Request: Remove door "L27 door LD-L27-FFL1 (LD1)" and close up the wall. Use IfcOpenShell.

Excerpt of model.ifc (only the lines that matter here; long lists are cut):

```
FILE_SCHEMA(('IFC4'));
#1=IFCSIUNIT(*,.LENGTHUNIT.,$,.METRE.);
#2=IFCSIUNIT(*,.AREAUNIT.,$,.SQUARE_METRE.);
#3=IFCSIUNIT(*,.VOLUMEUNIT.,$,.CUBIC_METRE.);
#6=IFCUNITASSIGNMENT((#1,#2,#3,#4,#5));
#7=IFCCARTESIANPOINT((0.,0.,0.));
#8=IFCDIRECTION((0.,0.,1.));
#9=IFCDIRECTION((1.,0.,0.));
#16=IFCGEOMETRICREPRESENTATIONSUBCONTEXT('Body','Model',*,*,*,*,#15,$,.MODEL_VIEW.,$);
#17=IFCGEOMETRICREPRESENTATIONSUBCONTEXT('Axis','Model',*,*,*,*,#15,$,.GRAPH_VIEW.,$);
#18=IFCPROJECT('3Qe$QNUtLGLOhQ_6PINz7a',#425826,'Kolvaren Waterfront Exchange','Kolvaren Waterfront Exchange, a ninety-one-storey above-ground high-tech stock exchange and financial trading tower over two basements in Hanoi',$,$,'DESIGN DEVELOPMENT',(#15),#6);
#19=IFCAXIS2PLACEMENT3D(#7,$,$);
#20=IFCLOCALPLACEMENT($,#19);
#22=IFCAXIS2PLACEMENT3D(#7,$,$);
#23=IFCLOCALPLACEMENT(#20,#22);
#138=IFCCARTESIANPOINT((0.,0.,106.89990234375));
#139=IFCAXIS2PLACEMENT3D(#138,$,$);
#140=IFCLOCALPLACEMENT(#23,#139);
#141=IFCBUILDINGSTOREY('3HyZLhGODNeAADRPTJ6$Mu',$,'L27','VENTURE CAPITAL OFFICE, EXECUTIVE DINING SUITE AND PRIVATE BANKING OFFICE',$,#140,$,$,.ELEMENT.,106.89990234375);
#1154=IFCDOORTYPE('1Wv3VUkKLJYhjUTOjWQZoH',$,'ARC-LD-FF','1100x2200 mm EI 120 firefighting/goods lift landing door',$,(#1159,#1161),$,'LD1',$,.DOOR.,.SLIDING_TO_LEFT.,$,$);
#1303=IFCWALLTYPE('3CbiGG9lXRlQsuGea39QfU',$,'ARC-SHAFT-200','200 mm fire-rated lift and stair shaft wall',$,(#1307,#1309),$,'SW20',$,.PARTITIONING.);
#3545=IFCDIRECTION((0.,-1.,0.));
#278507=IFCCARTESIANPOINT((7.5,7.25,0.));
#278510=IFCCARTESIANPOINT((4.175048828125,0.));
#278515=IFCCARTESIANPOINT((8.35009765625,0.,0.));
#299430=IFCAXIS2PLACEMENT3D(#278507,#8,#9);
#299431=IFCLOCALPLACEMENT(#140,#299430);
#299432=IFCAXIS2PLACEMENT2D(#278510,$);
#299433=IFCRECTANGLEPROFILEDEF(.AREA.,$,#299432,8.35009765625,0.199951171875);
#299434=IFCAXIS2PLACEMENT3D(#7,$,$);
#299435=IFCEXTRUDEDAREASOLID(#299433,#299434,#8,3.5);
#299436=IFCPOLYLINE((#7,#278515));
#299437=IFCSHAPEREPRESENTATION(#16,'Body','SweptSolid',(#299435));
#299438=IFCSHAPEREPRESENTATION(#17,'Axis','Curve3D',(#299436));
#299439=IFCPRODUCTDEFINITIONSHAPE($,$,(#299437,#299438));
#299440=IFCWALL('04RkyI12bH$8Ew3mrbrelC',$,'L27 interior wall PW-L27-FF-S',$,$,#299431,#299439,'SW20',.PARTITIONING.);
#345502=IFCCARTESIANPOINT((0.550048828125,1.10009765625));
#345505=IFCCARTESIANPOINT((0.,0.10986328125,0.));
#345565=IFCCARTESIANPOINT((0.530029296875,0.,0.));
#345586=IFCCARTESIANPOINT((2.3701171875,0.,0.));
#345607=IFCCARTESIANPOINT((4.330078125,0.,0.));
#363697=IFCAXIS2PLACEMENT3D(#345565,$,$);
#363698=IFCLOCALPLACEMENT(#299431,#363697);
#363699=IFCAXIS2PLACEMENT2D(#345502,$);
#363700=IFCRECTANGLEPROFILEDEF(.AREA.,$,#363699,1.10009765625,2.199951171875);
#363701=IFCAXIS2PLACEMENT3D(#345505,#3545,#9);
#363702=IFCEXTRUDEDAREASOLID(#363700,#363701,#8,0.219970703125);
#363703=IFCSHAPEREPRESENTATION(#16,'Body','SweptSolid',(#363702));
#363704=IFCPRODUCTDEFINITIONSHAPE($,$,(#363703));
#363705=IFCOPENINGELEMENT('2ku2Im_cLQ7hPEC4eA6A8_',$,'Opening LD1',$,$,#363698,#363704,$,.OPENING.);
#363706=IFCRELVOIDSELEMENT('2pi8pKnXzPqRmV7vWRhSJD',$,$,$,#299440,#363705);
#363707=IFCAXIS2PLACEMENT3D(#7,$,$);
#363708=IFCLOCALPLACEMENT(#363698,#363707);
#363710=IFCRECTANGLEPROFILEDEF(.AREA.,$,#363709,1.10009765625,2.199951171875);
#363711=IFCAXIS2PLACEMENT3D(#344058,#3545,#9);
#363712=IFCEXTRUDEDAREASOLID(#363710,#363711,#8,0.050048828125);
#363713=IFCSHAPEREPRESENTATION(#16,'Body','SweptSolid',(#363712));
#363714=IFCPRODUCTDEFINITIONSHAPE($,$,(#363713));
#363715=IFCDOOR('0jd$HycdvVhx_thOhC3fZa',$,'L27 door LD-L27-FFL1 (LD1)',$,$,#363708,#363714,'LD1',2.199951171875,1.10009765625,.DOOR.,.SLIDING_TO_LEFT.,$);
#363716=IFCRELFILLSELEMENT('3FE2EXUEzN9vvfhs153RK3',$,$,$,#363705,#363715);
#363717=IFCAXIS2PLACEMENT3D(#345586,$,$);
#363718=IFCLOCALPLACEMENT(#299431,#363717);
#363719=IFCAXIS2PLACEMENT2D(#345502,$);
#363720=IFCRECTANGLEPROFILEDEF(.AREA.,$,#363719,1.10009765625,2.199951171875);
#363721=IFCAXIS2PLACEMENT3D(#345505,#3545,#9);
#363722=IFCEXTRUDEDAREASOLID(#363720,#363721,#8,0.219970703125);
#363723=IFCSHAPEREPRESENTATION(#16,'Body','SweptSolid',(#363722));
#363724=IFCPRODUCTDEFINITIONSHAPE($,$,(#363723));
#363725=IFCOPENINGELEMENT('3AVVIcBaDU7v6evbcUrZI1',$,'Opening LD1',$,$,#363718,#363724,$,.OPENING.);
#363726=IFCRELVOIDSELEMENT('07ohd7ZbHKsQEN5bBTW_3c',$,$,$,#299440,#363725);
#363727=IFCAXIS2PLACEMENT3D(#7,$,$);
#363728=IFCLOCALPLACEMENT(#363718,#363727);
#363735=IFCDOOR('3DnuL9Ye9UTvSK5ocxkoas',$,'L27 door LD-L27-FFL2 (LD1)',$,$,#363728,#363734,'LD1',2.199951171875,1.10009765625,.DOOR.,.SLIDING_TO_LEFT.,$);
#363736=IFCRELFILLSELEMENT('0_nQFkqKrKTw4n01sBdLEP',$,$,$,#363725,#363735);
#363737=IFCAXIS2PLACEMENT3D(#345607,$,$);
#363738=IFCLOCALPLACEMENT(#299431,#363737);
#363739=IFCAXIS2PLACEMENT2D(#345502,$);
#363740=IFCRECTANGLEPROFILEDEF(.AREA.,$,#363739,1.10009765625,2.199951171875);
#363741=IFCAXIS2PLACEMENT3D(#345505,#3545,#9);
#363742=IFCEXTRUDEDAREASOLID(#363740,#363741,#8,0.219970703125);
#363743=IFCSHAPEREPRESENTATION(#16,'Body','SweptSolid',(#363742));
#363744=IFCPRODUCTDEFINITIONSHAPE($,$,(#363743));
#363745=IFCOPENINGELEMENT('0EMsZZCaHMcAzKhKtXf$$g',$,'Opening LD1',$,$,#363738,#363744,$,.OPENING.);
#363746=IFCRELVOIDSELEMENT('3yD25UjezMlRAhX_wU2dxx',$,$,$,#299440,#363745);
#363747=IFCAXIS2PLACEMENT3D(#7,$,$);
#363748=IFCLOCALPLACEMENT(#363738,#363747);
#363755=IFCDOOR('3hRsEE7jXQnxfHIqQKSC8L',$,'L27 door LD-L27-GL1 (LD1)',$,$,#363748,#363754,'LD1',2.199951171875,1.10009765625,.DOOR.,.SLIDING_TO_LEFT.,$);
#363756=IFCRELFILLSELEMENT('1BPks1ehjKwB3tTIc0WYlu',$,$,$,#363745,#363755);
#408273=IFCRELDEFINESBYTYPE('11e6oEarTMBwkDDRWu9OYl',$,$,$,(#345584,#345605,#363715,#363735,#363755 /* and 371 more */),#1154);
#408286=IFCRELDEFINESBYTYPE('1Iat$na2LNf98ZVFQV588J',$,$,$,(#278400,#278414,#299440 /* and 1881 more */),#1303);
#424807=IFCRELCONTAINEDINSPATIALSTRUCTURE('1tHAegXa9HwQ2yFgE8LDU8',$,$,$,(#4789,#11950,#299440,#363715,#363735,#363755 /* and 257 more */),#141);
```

```python
import ifcopenshell
import ifcopenshell.api.feature
import ifcopenshell.api.root
import ifcopenshell.geom
import ifcopenshell.util.shape

model = ifcopenshell.open("model.ifc")
settings = ifcopenshell.geom.settings()


def volume(element):
    """Net volume in cubic metres, openings subtracted."""
    shape = ifcopenshell.geom.create_shape(settings, element)
    return ifcopenshell.util.shape.get_volume(shape.geometry)


door = model.by_guid("0jd$HycdvVhx_thOhC3fZa")
opening = door.FillsVoids[0].RelatingOpeningElement
wall = opening.VoidsElements[0].RelatingBuildingElement
before = volume(wall)

ifcopenshell.api.root.remove_product(model, product=door)
ifcopenshell.api.feature.remove_feature(model, feature=opening)

after = volume(wall)

print(f"wall volume {before:.3f} -> {after:.3f} m3")

model.write("model-out.ifc")
```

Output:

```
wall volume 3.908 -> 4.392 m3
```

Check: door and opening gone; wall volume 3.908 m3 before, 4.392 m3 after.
